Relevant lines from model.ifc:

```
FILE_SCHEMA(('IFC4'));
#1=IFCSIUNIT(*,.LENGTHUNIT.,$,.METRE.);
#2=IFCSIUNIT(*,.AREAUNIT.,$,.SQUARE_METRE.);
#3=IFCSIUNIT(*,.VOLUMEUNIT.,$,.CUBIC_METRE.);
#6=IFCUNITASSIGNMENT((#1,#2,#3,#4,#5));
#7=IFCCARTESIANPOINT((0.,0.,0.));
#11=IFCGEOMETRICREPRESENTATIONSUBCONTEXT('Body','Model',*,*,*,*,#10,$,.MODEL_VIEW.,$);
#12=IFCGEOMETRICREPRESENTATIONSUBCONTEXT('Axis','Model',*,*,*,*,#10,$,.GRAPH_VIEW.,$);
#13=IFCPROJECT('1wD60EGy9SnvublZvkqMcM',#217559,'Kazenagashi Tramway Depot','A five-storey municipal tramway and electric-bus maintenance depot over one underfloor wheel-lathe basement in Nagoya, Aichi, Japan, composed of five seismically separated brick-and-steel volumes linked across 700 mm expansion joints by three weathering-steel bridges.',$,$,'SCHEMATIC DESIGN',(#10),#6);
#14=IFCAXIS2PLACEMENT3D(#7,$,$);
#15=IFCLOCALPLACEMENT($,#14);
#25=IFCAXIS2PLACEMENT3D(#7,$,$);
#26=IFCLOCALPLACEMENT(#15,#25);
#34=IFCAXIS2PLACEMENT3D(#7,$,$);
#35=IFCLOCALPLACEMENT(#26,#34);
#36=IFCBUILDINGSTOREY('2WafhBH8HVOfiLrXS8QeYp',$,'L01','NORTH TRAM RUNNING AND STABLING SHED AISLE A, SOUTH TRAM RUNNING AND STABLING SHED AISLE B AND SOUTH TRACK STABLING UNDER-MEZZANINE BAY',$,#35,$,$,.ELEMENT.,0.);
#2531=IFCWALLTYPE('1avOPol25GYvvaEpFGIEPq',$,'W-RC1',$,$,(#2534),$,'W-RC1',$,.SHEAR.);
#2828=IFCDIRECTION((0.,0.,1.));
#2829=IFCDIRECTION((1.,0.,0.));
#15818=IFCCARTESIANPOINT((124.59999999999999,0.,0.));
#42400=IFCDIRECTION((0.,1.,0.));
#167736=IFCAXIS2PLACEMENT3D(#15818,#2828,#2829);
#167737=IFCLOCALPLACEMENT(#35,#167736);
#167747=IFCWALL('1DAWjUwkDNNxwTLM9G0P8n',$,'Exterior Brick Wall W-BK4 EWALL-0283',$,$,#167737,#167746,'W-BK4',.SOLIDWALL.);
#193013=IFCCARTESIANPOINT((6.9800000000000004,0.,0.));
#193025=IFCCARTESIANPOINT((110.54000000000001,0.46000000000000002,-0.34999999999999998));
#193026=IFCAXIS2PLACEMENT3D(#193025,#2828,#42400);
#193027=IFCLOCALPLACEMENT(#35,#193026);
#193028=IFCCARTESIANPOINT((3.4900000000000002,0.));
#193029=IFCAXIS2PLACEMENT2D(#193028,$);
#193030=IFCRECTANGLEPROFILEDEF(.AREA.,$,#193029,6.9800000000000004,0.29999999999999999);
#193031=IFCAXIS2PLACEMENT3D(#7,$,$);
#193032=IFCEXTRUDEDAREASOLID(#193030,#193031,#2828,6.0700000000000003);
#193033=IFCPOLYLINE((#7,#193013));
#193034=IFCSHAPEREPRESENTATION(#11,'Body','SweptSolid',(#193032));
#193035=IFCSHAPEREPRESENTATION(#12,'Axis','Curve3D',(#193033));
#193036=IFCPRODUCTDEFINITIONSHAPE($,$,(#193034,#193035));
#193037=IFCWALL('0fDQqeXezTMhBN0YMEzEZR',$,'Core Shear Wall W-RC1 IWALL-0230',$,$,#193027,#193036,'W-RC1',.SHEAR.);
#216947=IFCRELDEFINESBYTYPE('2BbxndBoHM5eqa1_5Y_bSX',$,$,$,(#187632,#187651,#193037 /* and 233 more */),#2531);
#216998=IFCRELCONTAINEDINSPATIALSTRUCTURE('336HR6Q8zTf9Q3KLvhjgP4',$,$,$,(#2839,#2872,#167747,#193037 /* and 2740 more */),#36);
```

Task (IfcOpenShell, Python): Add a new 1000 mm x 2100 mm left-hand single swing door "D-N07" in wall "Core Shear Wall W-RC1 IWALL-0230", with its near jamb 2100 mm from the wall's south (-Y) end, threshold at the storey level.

```python
import numpy as np
import ifcopenshell
import ifcopenshell.api.feature
import ifcopenshell.api.geometry
import ifcopenshell.api.root
import ifcopenshell.api.spatial
import ifcopenshell.geom
import ifcopenshell.util.element
import ifcopenshell.util.placement
import ifcopenshell.util.representation
import ifcopenshell.util.shape
import ifcopenshell.util.unit

model = ifcopenshell.open("model.ifc")
unit_scale = ifcopenshell.util.unit.calculate_unit_scale(model)
settings = ifcopenshell.geom.settings()


def volume(element):
    """Net volume in cubic metres, openings subtracted."""
    shape = ifcopenshell.geom.create_shape(settings, element)
    return ifcopenshell.util.shape.get_volume(shape.geometry)


wall = model.by_guid("0fDQqeXezTMhBN0YMEzEZR")
storey = ifcopenshell.util.element.get_container(wall, ifc_class="IfcBuildingStorey")
context = ifcopenshell.util.representation.get_context(model, "Model", "Body", "MODEL_VIEW")
before = volume(wall)

width, height, from_end, sill = 1, 2.1, 2.1, 0.0  # metres

# The wall runs along its own X axis, and the end named is its -X end.
wall_shape = ifcopenshell.geom.create_shape(settings, wall)
x, y, z = ifcopenshell.util.shape.get_vertices(wall_shape.geometry).T
start = x.min() + from_end
face, thickness = float(y.min()), float(y.max() - y.min())
wall_matrix = ifcopenshell.util.placement.get_local_placement(wall.ObjectPlacement)
level = ifcopenshell.util.placement.get_local_placement(storey.ObjectPlacement)[2, 3]


def in_wall(x, y):
    """Placement at x, y metres in the wall's axes, at sill height."""
    matrix = wall_matrix.copy()
    matrix[:, 3] = wall_matrix @ np.array([x / unit_scale, y / unit_scale, 0.0, 1.0])
    matrix[2, 3] = level + sill / unit_scale
    return matrix


# Opening: a box that overshoots both wall faces by 50 mm.
opening = ifcopenshell.api.root.create_entity(model, ifc_class="IfcOpeningElement", predefined_type="OPENING")
box = ifcopenshell.api.geometry.add_wall_representation(
    model, context=context, length=width, height=height, thickness=thickness + 0.1
)
ifcopenshell.api.geometry.assign_representation(model, product=opening, representation=box)
ifcopenshell.api.geometry.edit_object_placement(model, product=opening, matrix=in_wall(start, face - 0.05), is_si=False)
ifcopenshell.api.feature.add_feature(model, feature=opening, element=wall)

door = ifcopenshell.api.root.create_entity(model, ifc_class="IfcDoor", name="D-N07", predefined_type="DOOR")
door.OverallWidth, door.OverallHeight = width / unit_scale, height / unit_scale
door.OperationType = "SINGLE_SWING_LEFT"
body = ifcopenshell.api.geometry.add_door_representation(
    model,
    context=context,
    overall_width=door.OverallWidth,
    overall_height=door.OverallHeight,
    operation_type="SINGLE_SWING_LEFT",
    lining_properties={"LiningDepth": thickness / unit_scale, "ThresholdDepth": thickness / unit_scale},
)
ifcopenshell.api.geometry.assign_representation(model, product=door, representation=body)
ifcopenshell.api.spatial.assign_container(model, products=[door], relating_structure=storey)
ifcopenshell.api.feature.add_filling(model, opening=opening, element=door)

# The lining spans the wall, so the door starts at the wall face.
ifcopenshell.api.geometry.edit_object_placement(model, product=door, matrix=in_wall(start, face), is_si=False)

after = volume(wall)

print(f"wall volume {before:.3f} -> {after:.3f} m3")

model.write("model_edited.ifc")
```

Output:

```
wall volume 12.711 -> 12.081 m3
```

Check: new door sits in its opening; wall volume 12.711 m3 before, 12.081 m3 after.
